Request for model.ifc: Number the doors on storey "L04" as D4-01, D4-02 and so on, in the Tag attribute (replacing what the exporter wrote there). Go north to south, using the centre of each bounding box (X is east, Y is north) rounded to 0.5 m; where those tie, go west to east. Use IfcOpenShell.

First a look at what the model holds.

```python
import ifcopenshell
import ifcopenshell.util.element
import ifcopenshell.util.placement

model = ifcopenshell.open("model.ifc")
print(model.schema)
storey = next(s for s in model.by_type("IfcBuildingStorey") if s.Name == "L04")
doors = [e for e in ifcopenshell.util.element.get_decomposition(storey) if e.is_a("IfcDoor")]
for e in sorted(doors, key=lambda e: e.id()):
    origin = ifcopenshell.util.placement.get_local_placement(e.ObjectPlacement)[:3, 3]
    print(e.id(), e.Tag, e.Name, origin.round(2) + 0.0, sep=" | ")
```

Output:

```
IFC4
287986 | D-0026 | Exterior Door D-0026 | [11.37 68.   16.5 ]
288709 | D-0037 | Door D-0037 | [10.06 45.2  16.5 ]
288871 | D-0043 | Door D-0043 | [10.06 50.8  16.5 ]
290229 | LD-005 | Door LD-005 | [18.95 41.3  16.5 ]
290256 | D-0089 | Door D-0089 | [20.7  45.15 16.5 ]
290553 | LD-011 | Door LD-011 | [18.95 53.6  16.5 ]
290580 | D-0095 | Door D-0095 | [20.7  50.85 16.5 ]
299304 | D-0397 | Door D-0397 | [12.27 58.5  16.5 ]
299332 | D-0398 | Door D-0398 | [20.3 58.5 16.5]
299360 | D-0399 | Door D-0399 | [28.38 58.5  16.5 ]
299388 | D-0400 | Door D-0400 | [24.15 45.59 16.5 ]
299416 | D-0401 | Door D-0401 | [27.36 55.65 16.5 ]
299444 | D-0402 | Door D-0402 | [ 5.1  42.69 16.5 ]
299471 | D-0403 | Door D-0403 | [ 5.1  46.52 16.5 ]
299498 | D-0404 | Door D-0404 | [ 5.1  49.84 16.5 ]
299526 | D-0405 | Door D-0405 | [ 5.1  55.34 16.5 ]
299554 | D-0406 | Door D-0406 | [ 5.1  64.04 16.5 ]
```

```python
import ifcopenshell
import ifcopenshell.geom
import ifcopenshell.util.element
import ifcopenshell.util.shape

model = ifcopenshell.open("model.ifc")
settings = ifcopenshell.geom.settings()
settings.set("use-world-coords", True)


def centre(element):
    shape = ifcopenshell.geom.create_shape(settings, element)
    return ifcopenshell.util.shape.get_bbox_centroid(shape.geometry)


storey = next(s for s in model.by_type("IfcBuildingStorey") if s.Name == "L04")
doors = [e for e in ifcopenshell.util.element.get_decomposition(storey) if e.is_a("IfcDoor")]

# Insertion points can sit at a corner or the storey origin, so sort by the geometry (in metres).
centres = {e: centre(e) for e in doors}
doors.sort(key=lambda e: (-round(centres[e][1] / 0.5), centres[e][0]))

for i, e in enumerate(doors, start=1):
    number = f"D4-{i:02d}"
    e.Tag = number
    print(e.id(), number)

model.write("model_v2.ifc")
```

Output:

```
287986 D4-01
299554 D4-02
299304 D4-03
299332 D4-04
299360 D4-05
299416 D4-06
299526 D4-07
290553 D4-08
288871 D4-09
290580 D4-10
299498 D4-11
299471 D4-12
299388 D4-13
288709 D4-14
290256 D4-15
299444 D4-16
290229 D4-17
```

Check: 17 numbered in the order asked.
